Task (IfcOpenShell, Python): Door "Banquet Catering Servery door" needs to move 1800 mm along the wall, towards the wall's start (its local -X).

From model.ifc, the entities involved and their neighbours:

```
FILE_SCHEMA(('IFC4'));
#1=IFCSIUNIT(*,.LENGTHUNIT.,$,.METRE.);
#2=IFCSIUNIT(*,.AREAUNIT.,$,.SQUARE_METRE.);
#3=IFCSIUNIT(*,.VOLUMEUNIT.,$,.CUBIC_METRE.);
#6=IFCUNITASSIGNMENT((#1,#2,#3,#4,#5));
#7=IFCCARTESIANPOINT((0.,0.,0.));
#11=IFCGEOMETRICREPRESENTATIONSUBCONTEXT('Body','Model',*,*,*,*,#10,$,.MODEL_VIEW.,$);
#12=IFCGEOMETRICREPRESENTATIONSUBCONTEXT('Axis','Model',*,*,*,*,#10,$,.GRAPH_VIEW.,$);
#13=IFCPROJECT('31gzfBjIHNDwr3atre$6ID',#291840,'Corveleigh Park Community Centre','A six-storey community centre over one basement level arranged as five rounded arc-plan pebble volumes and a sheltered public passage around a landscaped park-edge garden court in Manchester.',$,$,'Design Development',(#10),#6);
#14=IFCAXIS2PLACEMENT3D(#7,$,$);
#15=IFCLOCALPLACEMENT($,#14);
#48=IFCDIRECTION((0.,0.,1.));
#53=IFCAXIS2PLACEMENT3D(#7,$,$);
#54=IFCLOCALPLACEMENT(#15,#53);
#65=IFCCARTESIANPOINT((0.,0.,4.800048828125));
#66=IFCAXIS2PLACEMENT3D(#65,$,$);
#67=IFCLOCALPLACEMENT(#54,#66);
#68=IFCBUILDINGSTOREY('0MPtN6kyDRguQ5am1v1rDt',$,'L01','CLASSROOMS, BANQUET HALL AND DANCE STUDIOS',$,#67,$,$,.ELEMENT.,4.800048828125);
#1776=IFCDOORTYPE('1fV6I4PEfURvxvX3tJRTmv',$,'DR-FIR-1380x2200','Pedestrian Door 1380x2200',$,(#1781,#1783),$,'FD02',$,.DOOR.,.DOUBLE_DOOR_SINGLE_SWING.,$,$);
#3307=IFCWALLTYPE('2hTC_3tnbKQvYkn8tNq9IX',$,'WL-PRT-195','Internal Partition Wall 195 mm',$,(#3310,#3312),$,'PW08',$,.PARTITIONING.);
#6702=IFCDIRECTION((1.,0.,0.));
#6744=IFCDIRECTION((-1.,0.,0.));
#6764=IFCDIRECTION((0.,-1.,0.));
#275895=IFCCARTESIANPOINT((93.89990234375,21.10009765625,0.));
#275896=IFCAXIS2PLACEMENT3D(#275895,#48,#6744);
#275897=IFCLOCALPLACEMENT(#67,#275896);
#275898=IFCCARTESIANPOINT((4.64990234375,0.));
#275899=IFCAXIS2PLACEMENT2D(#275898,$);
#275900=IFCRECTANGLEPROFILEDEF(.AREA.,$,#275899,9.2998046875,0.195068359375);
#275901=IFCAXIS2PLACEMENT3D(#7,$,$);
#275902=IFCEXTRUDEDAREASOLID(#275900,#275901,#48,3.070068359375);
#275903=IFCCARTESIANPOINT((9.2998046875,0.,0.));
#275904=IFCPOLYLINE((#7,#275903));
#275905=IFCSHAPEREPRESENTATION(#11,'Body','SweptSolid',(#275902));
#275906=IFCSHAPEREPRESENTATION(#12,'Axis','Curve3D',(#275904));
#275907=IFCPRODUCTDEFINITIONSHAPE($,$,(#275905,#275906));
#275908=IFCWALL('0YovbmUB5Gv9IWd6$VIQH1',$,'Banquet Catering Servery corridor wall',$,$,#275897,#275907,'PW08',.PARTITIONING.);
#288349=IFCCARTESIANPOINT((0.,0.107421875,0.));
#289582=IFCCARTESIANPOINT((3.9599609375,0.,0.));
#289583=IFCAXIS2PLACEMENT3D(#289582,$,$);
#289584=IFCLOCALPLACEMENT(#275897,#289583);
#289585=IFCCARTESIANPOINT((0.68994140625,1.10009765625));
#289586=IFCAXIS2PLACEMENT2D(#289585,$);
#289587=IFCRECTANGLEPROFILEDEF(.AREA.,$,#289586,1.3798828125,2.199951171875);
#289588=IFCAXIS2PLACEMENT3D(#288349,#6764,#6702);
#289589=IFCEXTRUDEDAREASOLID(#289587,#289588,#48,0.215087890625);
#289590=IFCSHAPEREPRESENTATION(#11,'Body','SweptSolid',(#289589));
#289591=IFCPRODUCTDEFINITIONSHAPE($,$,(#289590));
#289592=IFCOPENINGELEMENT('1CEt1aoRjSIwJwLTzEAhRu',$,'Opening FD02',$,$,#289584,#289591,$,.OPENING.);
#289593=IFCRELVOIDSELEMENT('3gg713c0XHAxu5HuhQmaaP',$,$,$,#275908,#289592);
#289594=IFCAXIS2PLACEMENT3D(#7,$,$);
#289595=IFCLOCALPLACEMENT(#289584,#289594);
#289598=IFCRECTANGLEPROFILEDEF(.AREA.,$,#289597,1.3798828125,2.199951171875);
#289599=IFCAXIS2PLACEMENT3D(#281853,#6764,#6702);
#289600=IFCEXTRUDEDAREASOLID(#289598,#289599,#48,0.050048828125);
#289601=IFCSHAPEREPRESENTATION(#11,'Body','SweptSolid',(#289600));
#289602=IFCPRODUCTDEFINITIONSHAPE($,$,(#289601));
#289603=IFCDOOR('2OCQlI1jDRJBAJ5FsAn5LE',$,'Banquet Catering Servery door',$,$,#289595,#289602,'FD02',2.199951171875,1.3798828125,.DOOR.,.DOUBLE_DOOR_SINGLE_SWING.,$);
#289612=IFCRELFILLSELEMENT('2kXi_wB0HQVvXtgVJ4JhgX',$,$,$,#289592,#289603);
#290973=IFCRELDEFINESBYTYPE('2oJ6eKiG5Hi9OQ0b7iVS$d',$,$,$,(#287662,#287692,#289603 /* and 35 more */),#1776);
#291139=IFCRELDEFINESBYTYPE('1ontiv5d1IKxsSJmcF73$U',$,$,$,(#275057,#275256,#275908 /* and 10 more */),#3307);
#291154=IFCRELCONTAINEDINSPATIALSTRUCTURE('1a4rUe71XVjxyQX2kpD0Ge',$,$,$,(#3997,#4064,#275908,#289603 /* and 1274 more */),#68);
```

```python
import ifcopenshell
import ifcopenshell.api.geometry
import ifcopenshell.util.placement

model = ifcopenshell.open("model.ifc")

door = model.by_id(289603)
opening = door.FillsVoids[0].RelatingOpeningElement
wall = opening.VoidsElements[0].RelatingBuildingElement

wall_matrix = ifcopenshell.util.placement.get_local_placement(wall.ObjectPlacement)
shift = wall_matrix[:3, 0] * -1.8
before = ifcopenshell.util.placement.get_local_placement(door.ObjectPlacement)[:3, 3].copy()

# The door is placed relative to its opening, so it follows when the opening moves.
matrix = ifcopenshell.util.placement.get_local_placement(opening.ObjectPlacement)
matrix[:3, 3] += shift
ifcopenshell.api.geometry.edit_object_placement(
    model, product=opening, matrix=matrix, is_si=False, should_transform_children=True
)

after = ifcopenshell.util.placement.get_local_placement(door.ObjectPlacement)[:3, 3]
print("door moved by", (after - before).round(3) + 0.0)

model.write("model_edited.ifc")
```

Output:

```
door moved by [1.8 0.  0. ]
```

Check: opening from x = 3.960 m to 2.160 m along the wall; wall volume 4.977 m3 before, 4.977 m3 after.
